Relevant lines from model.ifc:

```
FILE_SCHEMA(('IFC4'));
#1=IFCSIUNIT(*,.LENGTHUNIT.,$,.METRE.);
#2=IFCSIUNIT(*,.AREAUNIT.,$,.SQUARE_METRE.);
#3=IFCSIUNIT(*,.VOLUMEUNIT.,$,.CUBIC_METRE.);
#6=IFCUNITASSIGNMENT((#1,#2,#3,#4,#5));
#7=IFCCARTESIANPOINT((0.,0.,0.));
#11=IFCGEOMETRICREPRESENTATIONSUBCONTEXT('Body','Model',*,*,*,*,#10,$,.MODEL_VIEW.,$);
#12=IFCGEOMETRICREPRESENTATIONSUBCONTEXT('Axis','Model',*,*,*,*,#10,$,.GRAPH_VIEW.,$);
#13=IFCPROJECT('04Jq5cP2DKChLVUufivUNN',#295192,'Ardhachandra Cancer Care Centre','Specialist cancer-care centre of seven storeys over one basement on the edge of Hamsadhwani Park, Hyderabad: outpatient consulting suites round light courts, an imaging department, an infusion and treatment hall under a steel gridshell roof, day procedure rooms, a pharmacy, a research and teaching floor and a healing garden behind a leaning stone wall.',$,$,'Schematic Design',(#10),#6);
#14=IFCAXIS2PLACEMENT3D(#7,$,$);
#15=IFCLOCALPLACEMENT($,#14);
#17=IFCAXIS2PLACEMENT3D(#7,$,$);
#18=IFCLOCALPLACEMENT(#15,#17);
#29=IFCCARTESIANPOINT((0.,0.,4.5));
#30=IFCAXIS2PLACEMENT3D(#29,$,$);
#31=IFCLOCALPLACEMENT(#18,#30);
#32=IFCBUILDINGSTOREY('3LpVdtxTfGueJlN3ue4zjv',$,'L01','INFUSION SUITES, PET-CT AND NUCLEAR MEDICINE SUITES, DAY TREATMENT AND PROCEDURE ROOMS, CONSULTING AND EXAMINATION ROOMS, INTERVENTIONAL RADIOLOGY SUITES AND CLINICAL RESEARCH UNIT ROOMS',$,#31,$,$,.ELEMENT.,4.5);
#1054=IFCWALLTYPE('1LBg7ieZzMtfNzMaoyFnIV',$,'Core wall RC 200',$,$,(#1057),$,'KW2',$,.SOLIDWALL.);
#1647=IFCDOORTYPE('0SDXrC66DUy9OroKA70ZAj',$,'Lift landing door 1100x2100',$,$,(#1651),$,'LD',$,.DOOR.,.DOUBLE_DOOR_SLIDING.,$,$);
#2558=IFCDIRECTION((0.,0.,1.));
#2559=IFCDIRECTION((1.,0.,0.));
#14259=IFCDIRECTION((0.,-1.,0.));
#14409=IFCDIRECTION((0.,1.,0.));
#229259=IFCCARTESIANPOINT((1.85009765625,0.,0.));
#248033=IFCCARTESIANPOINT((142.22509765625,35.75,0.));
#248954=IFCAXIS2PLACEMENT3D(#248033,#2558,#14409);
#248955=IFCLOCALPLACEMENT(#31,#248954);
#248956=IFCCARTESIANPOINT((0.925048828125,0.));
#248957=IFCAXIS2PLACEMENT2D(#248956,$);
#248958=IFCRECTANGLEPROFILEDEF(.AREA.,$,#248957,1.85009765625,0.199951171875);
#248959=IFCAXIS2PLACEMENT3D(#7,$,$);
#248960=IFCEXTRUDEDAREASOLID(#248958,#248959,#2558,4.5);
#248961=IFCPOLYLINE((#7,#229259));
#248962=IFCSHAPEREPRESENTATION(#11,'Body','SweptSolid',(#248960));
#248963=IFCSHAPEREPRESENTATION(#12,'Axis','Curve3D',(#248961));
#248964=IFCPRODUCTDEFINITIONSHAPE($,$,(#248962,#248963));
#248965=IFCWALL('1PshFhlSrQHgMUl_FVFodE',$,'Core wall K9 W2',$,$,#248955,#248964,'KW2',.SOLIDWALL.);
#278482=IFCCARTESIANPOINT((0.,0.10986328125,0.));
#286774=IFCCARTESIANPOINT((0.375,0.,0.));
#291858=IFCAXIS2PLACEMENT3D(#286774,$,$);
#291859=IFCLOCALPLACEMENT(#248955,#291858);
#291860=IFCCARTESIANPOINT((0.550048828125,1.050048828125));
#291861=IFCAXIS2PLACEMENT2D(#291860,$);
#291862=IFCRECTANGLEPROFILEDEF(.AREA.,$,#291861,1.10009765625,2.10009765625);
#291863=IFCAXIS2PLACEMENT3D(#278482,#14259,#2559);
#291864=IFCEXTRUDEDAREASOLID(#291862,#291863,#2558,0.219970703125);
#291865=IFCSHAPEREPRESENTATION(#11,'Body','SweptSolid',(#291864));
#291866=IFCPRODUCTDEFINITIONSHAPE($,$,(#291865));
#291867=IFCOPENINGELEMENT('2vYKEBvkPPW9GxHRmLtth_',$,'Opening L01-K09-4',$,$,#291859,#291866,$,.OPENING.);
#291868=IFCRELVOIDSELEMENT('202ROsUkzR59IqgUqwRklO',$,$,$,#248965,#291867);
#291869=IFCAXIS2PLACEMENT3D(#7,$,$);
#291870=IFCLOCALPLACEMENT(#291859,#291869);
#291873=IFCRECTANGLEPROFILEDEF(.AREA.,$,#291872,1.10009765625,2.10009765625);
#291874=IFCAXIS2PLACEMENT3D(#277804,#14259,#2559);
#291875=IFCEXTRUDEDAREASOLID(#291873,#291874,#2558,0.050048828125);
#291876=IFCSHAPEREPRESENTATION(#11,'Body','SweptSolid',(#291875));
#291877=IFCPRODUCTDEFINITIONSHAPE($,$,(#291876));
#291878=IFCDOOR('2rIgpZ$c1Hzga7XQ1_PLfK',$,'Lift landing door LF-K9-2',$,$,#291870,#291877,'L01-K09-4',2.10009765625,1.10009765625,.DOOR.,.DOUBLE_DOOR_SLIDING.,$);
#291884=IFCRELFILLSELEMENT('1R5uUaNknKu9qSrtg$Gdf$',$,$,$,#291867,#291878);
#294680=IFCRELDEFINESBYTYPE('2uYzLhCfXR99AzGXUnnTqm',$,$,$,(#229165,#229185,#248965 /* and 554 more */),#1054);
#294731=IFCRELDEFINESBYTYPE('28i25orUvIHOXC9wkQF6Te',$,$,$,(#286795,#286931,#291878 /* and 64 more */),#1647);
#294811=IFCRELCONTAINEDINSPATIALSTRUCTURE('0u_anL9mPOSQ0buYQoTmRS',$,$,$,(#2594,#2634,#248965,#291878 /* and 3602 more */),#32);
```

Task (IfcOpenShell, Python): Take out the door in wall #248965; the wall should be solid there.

```python
import ifcopenshell
import ifcopenshell.api.feature
import ifcopenshell.api.root
import ifcopenshell.geom
import ifcopenshell.util.shape

model = ifcopenshell.open("model.ifc")
settings = ifcopenshell.geom.settings()


def volume(element):
    """Net volume in cubic metres, openings subtracted."""
    shape = ifcopenshell.geom.create_shape(settings, element)
    return ifcopenshell.util.shape.get_volume(shape.geometry)


door = model.by_id(291878)
opening = door.FillsVoids[0].RelatingOpeningElement
wall = opening.VoidsElements[0].RelatingBuildingElement
before = volume(wall)

ifcopenshell.api.root.remove_product(model, product=door)
ifcopenshell.api.feature.remove_feature(model, feature=opening)

after = volume(wall)

print(f"wall volume {before:.3f} -> {after:.3f} m3")

model.write("model_updated.ifc")
```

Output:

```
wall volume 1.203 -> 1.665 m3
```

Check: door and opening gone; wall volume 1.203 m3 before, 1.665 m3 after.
